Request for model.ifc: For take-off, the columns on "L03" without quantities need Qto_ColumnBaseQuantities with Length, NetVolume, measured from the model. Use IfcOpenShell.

First a look at what the model holds.

```python
import ifcopenshell
import ifcopenshell.util.element
import ifcopenshell.util.unit

model = ifcopenshell.open("model.ifc")
print(model.schema)
for unit_type in ("LENGTHUNIT", "AREAUNIT", "VOLUMEUNIT"):
    print(unit_type, ifcopenshell.util.unit.calculate_unit_scale(model, unit_type))
storey = next(s for s in model.by_type("IfcBuildingStorey") if s.Name == "L03")
columns = [e for e in ifcopenshell.util.element.get_decomposition(storey) if e.is_a("IfcColumn")]
for e in sorted(columns, key=lambda e: e.id()):
    print(e.id(), e.is_a(), e.Name, list(ifcopenshell.util.element.get_psets(e, qtos_only=True)), sep=" | ")
```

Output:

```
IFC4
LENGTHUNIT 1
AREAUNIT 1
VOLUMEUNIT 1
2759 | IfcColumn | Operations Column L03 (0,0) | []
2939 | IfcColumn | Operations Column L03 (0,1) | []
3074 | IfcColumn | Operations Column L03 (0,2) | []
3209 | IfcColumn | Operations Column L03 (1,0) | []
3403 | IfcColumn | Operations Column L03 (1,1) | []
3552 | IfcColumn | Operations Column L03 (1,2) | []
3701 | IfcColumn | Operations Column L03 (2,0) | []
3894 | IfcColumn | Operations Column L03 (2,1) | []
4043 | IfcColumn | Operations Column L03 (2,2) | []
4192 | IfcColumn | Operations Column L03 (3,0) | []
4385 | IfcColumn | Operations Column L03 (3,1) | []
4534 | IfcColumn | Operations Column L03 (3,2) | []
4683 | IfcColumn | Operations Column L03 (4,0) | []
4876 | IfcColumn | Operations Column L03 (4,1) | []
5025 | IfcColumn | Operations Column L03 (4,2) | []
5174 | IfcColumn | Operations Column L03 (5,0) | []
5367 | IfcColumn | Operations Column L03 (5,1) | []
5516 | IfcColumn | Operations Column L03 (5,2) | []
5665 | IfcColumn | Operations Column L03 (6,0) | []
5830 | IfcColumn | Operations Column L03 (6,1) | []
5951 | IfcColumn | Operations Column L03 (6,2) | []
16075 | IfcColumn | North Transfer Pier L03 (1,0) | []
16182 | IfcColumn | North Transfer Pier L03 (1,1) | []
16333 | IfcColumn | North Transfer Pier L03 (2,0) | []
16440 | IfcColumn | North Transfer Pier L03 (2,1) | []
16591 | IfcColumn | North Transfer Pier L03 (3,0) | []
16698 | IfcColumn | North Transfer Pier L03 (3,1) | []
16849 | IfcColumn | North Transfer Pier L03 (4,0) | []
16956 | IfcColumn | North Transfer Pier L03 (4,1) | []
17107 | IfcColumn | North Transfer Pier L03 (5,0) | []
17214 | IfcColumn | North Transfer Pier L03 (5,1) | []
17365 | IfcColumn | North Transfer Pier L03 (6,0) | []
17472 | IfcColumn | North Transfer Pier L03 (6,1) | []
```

```python
import ifcopenshell
import ifcopenshell.api.pset
import ifcopenshell.geom
import ifcopenshell.util.element
import ifcopenshell.util.shape
import ifcopenshell.util.unit

model = ifcopenshell.open("model.ifc")
unit_scale = ifcopenshell.util.unit.calculate_unit_scale(model)
volume_scale = ifcopenshell.util.unit.calculate_unit_scale(model, "VOLUMEUNIT")
settings = ifcopenshell.geom.settings()

storey = next(s for s in model.by_type("IfcBuildingStorey") if s.Name == "L03")
columns = [e for e in ifcopenshell.util.element.get_decomposition(storey) if e.is_a("IfcColumn")]

for e in sorted(columns, key=lambda e: e.id()):
    if ifcopenshell.util.element.get_psets(e, qtos_only=True, should_inherit=False):
        continue
    # Geometry comes back in metres, in the element's own axes.
    shape = ifcopenshell.geom.create_shape(settings, e)
    values = {
        "Length": ifcopenshell.util.shape.get_z(shape.geometry) / unit_scale,
        "NetVolume": ifcopenshell.util.shape.get_volume(shape.geometry) / volume_scale,
    }
    qto = ifcopenshell.api.pset.add_qto(model, product=e, name="Qto_ColumnBaseQuantities")
    ifcopenshell.api.pset.edit_qto(model, qto=qto, properties=values)
    print(e.id(), {k: round(v, 3) for k, v in values.items()})

model.write("model_updated.ifc")
```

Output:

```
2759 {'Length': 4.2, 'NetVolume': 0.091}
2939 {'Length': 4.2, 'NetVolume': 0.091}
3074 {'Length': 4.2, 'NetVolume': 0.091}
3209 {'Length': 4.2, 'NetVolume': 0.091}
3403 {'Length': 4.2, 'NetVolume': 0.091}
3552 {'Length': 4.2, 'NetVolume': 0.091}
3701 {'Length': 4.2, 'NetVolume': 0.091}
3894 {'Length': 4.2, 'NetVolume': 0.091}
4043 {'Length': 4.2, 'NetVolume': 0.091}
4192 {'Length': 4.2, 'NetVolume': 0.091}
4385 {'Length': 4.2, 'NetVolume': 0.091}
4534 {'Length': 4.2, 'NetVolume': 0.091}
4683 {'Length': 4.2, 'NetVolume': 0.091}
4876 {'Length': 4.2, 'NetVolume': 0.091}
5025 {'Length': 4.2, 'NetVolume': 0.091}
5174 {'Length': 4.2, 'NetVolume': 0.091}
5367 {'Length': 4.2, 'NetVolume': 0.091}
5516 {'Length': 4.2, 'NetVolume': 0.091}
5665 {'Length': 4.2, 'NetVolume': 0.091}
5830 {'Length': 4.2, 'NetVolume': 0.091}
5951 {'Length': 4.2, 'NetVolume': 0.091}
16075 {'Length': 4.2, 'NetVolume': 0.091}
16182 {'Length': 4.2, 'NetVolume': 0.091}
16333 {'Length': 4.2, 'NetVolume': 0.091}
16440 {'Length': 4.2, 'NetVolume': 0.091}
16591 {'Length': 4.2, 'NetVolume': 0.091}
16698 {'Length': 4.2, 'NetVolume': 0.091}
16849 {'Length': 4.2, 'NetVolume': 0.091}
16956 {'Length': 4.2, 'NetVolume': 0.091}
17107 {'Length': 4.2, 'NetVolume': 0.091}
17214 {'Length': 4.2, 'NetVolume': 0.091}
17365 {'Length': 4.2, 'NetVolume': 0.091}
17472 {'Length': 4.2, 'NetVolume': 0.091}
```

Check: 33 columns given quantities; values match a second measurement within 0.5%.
